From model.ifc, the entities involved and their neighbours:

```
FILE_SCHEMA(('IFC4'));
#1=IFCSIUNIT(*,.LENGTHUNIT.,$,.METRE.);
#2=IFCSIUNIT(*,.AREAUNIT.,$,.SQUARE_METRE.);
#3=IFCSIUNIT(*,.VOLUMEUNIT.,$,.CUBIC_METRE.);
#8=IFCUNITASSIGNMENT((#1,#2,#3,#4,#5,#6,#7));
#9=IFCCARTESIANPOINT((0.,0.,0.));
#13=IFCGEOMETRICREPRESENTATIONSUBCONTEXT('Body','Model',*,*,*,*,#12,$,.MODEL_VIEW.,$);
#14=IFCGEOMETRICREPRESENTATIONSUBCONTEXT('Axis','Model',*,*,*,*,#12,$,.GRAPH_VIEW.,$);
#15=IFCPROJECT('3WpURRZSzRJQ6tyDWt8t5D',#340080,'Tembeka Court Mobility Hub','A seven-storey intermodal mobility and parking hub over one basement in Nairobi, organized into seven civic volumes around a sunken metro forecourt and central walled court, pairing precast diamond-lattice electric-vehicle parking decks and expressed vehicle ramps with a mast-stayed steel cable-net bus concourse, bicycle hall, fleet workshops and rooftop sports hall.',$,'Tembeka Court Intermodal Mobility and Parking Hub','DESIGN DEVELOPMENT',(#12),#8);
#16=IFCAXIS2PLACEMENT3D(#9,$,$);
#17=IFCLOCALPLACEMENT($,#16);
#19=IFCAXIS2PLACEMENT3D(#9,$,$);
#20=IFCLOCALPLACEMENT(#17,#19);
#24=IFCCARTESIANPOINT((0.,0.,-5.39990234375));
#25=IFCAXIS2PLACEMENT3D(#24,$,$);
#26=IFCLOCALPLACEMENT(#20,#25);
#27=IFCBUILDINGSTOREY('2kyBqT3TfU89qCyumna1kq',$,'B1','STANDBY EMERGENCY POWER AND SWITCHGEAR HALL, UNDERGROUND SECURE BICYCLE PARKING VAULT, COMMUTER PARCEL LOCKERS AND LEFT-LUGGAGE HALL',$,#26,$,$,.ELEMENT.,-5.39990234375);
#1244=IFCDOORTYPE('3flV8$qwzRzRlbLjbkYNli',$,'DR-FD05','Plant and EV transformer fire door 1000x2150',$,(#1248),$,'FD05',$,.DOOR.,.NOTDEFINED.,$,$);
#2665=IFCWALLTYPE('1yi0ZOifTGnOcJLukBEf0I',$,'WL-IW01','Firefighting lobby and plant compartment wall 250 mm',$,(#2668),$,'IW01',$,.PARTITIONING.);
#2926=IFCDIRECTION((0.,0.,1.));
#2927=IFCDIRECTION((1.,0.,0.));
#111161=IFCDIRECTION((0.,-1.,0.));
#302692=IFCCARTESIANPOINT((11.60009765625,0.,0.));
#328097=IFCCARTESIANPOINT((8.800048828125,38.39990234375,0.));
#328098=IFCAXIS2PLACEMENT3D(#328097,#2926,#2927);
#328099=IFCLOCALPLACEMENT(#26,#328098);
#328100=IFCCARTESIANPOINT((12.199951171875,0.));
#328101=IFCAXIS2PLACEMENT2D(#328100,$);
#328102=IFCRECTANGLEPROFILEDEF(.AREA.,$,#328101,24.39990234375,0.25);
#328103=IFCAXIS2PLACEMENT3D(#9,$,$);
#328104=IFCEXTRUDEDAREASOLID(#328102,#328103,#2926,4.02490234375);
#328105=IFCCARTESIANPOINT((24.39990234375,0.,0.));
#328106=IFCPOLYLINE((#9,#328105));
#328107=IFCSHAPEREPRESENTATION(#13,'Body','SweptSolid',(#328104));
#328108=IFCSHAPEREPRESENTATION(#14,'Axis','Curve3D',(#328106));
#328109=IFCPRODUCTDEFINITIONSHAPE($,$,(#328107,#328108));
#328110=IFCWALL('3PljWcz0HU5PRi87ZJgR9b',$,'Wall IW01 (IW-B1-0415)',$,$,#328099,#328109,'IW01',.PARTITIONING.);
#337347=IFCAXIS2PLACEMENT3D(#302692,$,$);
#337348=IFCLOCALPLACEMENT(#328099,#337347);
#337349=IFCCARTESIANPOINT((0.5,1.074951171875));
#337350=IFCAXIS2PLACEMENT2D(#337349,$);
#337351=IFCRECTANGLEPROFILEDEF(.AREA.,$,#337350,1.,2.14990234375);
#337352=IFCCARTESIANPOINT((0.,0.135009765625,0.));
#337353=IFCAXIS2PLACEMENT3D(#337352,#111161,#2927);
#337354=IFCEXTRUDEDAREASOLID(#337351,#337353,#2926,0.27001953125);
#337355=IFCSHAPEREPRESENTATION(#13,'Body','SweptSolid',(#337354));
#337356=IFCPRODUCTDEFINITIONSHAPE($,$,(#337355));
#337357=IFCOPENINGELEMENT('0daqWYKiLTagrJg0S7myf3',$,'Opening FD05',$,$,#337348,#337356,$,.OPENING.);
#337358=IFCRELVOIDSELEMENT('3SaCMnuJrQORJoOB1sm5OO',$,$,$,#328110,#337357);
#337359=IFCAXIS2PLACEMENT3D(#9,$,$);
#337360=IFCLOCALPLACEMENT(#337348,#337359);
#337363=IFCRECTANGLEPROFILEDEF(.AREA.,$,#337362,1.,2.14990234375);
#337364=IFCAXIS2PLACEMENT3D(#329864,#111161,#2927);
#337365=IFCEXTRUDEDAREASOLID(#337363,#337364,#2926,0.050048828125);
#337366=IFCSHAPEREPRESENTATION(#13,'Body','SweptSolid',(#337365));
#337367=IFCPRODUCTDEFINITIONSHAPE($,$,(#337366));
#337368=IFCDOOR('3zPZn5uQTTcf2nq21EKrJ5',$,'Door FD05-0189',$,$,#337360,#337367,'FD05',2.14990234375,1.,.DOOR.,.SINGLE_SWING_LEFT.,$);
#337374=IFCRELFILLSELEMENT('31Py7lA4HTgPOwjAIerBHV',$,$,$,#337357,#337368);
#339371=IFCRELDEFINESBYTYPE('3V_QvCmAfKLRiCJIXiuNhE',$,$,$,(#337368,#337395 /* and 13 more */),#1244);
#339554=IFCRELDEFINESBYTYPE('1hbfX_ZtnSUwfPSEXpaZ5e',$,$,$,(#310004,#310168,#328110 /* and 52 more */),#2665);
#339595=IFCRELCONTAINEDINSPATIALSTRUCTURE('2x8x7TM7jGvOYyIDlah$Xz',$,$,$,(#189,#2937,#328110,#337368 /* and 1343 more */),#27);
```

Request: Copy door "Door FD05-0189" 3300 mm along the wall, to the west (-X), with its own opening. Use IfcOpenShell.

```python
import ifcopenshell
import ifcopenshell.api.feature
import ifcopenshell.api.geometry
import ifcopenshell.api.root
import ifcopenshell.geom
import ifcopenshell.util.element
import ifcopenshell.util.placement
import ifcopenshell.util.shape
import ifcopenshell.util.unit

model = ifcopenshell.open("model.ifc")
unit_scale = ifcopenshell.util.unit.calculate_unit_scale(model)
settings = ifcopenshell.geom.settings()


def volume(element):
    """Net volume in cubic metres, openings subtracted."""
    shape = ifcopenshell.geom.create_shape(settings, element)
    return ifcopenshell.util.shape.get_volume(shape.geometry)


door = model.by_guid("3zPZn5uQTTcf2nq21EKrJ5")
opening = door.FillsVoids[0].RelatingOpeningElement
wall = opening.VoidsElements[0].RelatingBuildingElement
before = volume(wall)
shift = ifcopenshell.util.placement.get_local_placement(wall.ObjectPlacement)[:3, 0] * -3.3 / unit_scale

# copy_class copies the void relationship, type, container and properties, but no geometry.
new_opening = ifcopenshell.api.root.copy_class(model, product=opening)
new_opening.Representation = ifcopenshell.util.element.copy_deep(
    model, opening.Representation, exclude=["IfcGeometricRepresentationContext", "IfcRepresentationMap"]
)
new_door = ifcopenshell.api.root.copy_class(model, product=door)
new_door.Representation = ifcopenshell.util.element.copy_deep(
    model, door.Representation, exclude=["IfcGeometricRepresentationContext", "IfcRepresentationMap"]
)
new_door.Tag = None
ifcopenshell.api.feature.add_filling(model, opening=new_opening, element=new_door)

for old, new in ((opening, new_opening), (door, new_door)):
    matrix = ifcopenshell.util.placement.get_local_placement(old.ObjectPlacement)
    matrix[:3, 3] += shift
    ifcopenshell.api.geometry.edit_object_placement(model, product=new, matrix=matrix, is_si=False)

after = volume(wall)

print(f"wall volume {before:.3f} -> {after:.3f} m3")

model.write("model_edited.ifc")
```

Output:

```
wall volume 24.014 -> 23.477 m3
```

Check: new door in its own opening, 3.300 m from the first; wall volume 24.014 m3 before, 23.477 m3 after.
